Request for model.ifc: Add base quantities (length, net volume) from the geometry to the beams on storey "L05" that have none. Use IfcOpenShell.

First a look at what the model holds.

```python
import ifcopenshell
import ifcopenshell.util.element
import ifcopenshell.util.unit

model = ifcopenshell.open("model.ifc")
print(model.schema)
for unit_type in ("LENGTHUNIT", "AREAUNIT", "VOLUMEUNIT"):
    print(unit_type, ifcopenshell.util.unit.calculate_unit_scale(model, unit_type))
storey = next(s for s in model.by_type("IfcBuildingStorey") if s.Name == "L05")
beams = [e for e in ifcopenshell.util.element.get_decomposition(storey) if e.is_a("IfcBeam")]
for e in sorted(beams, key=lambda e: e.id()):
    print(e.id(), e.is_a(), e.Name, list(ifcopenshell.util.element.get_psets(e, qtos_only=True)), sep=" | ")
```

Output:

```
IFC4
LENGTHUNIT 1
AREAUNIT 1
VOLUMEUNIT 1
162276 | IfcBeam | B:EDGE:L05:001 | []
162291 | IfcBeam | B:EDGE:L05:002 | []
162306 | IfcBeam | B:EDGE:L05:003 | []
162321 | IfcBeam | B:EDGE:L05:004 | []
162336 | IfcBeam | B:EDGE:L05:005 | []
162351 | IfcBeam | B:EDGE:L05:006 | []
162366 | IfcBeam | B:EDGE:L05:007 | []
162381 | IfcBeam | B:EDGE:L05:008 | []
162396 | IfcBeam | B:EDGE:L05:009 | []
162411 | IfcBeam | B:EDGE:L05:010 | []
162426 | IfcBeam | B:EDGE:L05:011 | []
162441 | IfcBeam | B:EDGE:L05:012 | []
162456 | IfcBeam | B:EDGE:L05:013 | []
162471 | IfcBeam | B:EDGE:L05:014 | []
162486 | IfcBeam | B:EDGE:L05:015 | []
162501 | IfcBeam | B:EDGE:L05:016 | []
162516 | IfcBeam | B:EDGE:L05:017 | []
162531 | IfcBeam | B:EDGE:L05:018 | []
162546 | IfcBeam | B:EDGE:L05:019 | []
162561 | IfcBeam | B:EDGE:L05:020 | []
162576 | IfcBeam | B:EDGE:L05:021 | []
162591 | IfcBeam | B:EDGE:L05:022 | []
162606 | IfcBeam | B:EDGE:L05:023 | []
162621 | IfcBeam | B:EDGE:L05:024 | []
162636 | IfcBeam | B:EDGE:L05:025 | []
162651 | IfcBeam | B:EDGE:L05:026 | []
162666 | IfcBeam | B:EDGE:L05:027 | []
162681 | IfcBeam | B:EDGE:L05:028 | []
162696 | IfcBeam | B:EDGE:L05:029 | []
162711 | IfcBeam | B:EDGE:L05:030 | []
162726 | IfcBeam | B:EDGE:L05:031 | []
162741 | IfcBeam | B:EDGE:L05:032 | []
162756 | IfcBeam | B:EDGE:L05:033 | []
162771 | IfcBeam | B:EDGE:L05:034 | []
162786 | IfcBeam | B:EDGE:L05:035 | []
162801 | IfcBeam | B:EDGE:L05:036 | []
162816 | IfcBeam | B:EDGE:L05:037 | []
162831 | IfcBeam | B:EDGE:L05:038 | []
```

```python
import ifcopenshell
import ifcopenshell.api.pset
import ifcopenshell.geom
import ifcopenshell.util.element
import ifcopenshell.util.shape
import ifcopenshell.util.unit

model = ifcopenshell.open("model.ifc")
unit_scale = ifcopenshell.util.unit.calculate_unit_scale(model)
volume_scale = ifcopenshell.util.unit.calculate_unit_scale(model, "VOLUMEUNIT")
settings = ifcopenshell.geom.settings()

storey = next(s for s in model.by_type("IfcBuildingStorey") if s.Name == "L05")
beams = [e for e in ifcopenshell.util.element.get_decomposition(storey) if e.is_a("IfcBeam")]

for e in sorted(beams, key=lambda e: e.id()):
    if ifcopenshell.util.element.get_psets(e, qtos_only=True, should_inherit=False):
        continue
    # Geometry comes back in metres, in the element's own axes.
    shape = ifcopenshell.geom.create_shape(settings, e)
    values = {
        "Length": ifcopenshell.util.shape.get_max_xyz(shape.geometry) / unit_scale,
        "NetVolume": ifcopenshell.util.shape.get_volume(shape.geometry) / volume_scale,
    }
    qto = ifcopenshell.api.pset.add_qto(model, product=e, name="Qto_BeamBaseQuantities")
    ifcopenshell.api.pset.edit_qto(model, qto=qto, properties=values)
    print(e.id(), {k: round(v, 3) for k, v in values.items()})

model.write("model_rev.ifc")
```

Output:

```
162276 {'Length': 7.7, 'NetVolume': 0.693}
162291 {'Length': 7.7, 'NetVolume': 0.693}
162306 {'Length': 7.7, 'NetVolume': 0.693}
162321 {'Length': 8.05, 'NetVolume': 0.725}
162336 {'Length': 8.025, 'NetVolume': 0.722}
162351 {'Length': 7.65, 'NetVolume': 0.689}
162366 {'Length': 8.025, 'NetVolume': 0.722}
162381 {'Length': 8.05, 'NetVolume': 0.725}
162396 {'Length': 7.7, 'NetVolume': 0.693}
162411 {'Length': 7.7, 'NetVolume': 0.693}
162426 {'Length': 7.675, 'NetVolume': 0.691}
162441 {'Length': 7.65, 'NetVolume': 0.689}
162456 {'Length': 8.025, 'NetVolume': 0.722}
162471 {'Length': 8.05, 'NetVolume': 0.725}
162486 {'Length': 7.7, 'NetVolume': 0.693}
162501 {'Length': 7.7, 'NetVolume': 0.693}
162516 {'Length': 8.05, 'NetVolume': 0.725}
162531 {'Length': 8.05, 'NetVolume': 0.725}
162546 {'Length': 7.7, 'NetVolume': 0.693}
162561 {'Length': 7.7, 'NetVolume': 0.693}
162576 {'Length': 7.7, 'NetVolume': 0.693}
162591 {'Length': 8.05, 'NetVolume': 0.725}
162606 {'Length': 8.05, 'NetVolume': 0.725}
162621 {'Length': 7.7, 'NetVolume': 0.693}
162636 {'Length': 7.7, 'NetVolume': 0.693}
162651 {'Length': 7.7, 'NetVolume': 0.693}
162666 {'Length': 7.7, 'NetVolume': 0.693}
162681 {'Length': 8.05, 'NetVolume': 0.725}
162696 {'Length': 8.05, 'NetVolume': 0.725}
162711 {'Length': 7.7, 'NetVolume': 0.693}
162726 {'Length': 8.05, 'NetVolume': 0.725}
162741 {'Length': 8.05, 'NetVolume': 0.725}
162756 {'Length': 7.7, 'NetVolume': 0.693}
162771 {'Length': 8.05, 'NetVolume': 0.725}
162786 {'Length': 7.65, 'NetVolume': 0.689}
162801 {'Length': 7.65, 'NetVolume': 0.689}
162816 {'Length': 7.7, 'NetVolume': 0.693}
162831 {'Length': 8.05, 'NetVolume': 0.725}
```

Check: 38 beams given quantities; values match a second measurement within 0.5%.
